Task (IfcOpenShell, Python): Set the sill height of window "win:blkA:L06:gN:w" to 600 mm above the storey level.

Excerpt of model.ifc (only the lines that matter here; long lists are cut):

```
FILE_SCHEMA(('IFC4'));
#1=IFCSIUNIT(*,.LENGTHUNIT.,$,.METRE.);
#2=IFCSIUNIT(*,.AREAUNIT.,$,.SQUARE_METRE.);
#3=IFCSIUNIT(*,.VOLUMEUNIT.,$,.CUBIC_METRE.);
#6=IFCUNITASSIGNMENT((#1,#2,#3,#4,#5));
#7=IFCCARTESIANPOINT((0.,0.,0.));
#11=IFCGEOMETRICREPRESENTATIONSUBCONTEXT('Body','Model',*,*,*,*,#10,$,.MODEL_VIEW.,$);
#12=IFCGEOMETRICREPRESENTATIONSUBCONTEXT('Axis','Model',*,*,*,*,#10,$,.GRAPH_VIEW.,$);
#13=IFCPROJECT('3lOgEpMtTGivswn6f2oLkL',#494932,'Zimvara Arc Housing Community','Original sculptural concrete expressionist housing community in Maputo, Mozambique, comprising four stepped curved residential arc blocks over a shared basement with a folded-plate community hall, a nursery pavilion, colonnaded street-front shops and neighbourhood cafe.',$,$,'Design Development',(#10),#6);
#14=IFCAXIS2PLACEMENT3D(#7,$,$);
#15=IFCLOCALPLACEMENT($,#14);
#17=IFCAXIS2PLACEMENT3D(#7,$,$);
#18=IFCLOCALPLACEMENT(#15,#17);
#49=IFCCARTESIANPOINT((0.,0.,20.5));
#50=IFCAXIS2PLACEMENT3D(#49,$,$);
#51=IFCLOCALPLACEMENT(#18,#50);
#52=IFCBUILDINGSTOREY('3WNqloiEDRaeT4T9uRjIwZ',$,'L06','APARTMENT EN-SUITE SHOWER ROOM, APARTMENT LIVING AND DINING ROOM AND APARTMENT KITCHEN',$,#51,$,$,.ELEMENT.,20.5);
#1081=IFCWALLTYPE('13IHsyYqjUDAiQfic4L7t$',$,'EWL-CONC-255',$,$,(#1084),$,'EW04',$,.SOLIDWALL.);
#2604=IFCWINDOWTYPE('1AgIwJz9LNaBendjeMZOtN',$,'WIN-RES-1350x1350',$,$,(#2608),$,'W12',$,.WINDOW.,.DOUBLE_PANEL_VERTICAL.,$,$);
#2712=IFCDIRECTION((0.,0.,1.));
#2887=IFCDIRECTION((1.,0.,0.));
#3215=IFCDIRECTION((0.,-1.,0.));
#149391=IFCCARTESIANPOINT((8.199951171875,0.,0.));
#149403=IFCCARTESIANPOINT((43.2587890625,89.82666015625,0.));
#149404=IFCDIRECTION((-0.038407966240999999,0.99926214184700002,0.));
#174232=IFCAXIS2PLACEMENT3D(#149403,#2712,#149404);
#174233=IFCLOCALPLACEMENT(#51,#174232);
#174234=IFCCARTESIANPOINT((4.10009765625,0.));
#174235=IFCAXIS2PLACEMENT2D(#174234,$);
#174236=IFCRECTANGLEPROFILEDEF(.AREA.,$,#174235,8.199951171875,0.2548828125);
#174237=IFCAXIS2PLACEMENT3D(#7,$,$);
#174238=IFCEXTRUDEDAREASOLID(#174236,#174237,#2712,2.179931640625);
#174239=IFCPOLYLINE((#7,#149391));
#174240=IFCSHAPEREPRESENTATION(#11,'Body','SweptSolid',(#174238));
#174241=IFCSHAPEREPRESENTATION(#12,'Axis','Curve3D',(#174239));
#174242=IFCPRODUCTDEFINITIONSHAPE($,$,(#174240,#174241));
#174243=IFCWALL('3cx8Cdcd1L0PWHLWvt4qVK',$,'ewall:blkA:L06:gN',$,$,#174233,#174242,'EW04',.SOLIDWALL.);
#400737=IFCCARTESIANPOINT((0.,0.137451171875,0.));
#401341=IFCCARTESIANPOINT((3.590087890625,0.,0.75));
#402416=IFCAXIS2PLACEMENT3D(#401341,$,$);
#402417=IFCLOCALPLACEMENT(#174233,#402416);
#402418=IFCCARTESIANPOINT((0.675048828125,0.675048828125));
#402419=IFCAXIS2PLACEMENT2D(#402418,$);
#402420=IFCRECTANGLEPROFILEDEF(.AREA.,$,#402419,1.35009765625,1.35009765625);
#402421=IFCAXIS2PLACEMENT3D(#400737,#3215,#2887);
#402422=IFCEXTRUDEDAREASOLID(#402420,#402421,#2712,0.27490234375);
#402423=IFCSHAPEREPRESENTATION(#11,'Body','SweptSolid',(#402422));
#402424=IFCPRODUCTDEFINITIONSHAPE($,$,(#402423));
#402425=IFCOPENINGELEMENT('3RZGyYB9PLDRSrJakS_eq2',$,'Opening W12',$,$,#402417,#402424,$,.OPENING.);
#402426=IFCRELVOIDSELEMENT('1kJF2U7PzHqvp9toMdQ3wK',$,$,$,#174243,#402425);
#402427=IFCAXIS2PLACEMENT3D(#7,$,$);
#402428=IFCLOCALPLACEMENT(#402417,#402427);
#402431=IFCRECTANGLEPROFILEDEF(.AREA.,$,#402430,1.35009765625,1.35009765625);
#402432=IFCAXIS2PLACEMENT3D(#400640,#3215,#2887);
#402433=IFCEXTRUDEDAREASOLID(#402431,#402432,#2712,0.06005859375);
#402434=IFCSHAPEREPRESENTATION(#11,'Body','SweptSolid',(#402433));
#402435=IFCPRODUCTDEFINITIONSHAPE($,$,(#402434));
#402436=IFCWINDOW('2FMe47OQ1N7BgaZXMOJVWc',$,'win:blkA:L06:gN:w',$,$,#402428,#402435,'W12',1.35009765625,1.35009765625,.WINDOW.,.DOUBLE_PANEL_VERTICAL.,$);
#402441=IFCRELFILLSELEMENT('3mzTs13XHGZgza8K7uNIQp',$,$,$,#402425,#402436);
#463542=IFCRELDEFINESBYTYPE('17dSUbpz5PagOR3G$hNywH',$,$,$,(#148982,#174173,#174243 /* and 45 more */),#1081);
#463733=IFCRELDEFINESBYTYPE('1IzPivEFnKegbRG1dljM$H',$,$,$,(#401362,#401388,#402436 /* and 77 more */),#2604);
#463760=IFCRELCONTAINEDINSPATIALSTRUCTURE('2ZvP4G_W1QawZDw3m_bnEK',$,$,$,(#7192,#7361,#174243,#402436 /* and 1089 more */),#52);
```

```python
import numpy as np
import ifcopenshell
import ifcopenshell.api.geometry
import ifcopenshell.geom
import ifcopenshell.util.element
import ifcopenshell.util.placement
import ifcopenshell.util.shape
import ifcopenshell.util.unit

model = ifcopenshell.open("model.ifc")
unit_scale = ifcopenshell.util.unit.calculate_unit_scale(model)

window = model.by_id(402436)
opening = window.FillsVoids[0].RelatingOpeningElement
storey = ifcopenshell.util.element.get_container(window, ifc_class="IfcBuildingStorey")
level = ifcopenshell.util.placement.get_local_placement(storey.ObjectPlacement)[2, 3]

# The opening's origin need not be at the sill, so measure its lowest point.
shape = ifcopenshell.geom.create_shape(ifcopenshell.geom.settings(), opening)
bottom = ifcopenshell.util.shape.get_shape_bottom_elevation(shape, shape.geometry) / unit_scale
dz = level + 0.6 - bottom

shift = np.array([0.0, 0.0, dz])
# The window is placed relative to its opening, so it follows when the opening moves.
matrix = ifcopenshell.util.placement.get_local_placement(opening.ObjectPlacement)
matrix[:3, 3] += shift
ifcopenshell.api.geometry.edit_object_placement(
    model, product=opening, matrix=matrix, is_si=False, should_transform_children=True
)

print(f"moved by {dz * unit_scale:+.3f} m")

model.write("model_edited.ifc")
```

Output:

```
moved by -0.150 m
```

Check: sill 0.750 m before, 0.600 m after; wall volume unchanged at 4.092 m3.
